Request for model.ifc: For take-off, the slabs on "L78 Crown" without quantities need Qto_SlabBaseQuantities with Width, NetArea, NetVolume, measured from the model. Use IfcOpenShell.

First a look at what the model holds.

```python
import ifcopenshell
import ifcopenshell.util.element
import ifcopenshell.util.unit

model = ifcopenshell.open("model.ifc")
print(model.schema)
for unit_type in ("LENGTHUNIT", "AREAUNIT", "VOLUMEUNIT"):
    print(unit_type, ifcopenshell.util.unit.calculate_unit_scale(model, unit_type))
storey = next(s for s in model.by_type("IfcBuildingStorey") if s.Name == "L78 Crown")
slabs = [e for e in ifcopenshell.util.element.get_decomposition(storey) if e.is_a("IfcSlab")]
for e in sorted(slabs, key=lambda e: e.id()):
    print(e.id(), e.is_a(), e.Name, list(ifcopenshell.util.element.get_psets(e, qtos_only=True)), sep=" | ")
```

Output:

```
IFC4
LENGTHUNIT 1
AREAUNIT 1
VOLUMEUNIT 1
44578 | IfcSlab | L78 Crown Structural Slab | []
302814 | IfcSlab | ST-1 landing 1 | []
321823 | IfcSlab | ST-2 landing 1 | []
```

```python
import ifcopenshell
import ifcopenshell.api.pset
import ifcopenshell.geom
import ifcopenshell.util.element
import ifcopenshell.util.shape
import ifcopenshell.util.unit

model = ifcopenshell.open("model.ifc")
unit_scale = ifcopenshell.util.unit.calculate_unit_scale(model)
area_scale = ifcopenshell.util.unit.calculate_unit_scale(model, "AREAUNIT")
volume_scale = ifcopenshell.util.unit.calculate_unit_scale(model, "VOLUMEUNIT")
settings = ifcopenshell.geom.settings()

storey = next(s for s in model.by_type("IfcBuildingStorey") if s.Name == "L78 Crown")
slabs = [e for e in ifcopenshell.util.element.get_decomposition(storey) if e.is_a("IfcSlab")]

for e in sorted(slabs, key=lambda e: e.id()):
    if ifcopenshell.util.element.get_psets(e, qtos_only=True, should_inherit=False):
        continue
    # Geometry comes back in metres, in the element's own axes.
    shape = ifcopenshell.geom.create_shape(settings, e)
    values = {
        "Width": ifcopenshell.util.shape.get_z(shape.geometry) / unit_scale,
        "NetArea": ifcopenshell.util.shape.get_footprint_area(shape.geometry) / area_scale,
        "NetVolume": ifcopenshell.util.shape.get_volume(shape.geometry) / volume_scale,
    }
    qto = ifcopenshell.api.pset.add_qto(model, product=e, name="Qto_SlabBaseQuantities")
    ifcopenshell.api.pset.edit_qto(model, qto=qto, properties=values)
    print(e.id(), {k: round(v, 3) for k, v in values.items()})

model.write("model_edited.ifc")
```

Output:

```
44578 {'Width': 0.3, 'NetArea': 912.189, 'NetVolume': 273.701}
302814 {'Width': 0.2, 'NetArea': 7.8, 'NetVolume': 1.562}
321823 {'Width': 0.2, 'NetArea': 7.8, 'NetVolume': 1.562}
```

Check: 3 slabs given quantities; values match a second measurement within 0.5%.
